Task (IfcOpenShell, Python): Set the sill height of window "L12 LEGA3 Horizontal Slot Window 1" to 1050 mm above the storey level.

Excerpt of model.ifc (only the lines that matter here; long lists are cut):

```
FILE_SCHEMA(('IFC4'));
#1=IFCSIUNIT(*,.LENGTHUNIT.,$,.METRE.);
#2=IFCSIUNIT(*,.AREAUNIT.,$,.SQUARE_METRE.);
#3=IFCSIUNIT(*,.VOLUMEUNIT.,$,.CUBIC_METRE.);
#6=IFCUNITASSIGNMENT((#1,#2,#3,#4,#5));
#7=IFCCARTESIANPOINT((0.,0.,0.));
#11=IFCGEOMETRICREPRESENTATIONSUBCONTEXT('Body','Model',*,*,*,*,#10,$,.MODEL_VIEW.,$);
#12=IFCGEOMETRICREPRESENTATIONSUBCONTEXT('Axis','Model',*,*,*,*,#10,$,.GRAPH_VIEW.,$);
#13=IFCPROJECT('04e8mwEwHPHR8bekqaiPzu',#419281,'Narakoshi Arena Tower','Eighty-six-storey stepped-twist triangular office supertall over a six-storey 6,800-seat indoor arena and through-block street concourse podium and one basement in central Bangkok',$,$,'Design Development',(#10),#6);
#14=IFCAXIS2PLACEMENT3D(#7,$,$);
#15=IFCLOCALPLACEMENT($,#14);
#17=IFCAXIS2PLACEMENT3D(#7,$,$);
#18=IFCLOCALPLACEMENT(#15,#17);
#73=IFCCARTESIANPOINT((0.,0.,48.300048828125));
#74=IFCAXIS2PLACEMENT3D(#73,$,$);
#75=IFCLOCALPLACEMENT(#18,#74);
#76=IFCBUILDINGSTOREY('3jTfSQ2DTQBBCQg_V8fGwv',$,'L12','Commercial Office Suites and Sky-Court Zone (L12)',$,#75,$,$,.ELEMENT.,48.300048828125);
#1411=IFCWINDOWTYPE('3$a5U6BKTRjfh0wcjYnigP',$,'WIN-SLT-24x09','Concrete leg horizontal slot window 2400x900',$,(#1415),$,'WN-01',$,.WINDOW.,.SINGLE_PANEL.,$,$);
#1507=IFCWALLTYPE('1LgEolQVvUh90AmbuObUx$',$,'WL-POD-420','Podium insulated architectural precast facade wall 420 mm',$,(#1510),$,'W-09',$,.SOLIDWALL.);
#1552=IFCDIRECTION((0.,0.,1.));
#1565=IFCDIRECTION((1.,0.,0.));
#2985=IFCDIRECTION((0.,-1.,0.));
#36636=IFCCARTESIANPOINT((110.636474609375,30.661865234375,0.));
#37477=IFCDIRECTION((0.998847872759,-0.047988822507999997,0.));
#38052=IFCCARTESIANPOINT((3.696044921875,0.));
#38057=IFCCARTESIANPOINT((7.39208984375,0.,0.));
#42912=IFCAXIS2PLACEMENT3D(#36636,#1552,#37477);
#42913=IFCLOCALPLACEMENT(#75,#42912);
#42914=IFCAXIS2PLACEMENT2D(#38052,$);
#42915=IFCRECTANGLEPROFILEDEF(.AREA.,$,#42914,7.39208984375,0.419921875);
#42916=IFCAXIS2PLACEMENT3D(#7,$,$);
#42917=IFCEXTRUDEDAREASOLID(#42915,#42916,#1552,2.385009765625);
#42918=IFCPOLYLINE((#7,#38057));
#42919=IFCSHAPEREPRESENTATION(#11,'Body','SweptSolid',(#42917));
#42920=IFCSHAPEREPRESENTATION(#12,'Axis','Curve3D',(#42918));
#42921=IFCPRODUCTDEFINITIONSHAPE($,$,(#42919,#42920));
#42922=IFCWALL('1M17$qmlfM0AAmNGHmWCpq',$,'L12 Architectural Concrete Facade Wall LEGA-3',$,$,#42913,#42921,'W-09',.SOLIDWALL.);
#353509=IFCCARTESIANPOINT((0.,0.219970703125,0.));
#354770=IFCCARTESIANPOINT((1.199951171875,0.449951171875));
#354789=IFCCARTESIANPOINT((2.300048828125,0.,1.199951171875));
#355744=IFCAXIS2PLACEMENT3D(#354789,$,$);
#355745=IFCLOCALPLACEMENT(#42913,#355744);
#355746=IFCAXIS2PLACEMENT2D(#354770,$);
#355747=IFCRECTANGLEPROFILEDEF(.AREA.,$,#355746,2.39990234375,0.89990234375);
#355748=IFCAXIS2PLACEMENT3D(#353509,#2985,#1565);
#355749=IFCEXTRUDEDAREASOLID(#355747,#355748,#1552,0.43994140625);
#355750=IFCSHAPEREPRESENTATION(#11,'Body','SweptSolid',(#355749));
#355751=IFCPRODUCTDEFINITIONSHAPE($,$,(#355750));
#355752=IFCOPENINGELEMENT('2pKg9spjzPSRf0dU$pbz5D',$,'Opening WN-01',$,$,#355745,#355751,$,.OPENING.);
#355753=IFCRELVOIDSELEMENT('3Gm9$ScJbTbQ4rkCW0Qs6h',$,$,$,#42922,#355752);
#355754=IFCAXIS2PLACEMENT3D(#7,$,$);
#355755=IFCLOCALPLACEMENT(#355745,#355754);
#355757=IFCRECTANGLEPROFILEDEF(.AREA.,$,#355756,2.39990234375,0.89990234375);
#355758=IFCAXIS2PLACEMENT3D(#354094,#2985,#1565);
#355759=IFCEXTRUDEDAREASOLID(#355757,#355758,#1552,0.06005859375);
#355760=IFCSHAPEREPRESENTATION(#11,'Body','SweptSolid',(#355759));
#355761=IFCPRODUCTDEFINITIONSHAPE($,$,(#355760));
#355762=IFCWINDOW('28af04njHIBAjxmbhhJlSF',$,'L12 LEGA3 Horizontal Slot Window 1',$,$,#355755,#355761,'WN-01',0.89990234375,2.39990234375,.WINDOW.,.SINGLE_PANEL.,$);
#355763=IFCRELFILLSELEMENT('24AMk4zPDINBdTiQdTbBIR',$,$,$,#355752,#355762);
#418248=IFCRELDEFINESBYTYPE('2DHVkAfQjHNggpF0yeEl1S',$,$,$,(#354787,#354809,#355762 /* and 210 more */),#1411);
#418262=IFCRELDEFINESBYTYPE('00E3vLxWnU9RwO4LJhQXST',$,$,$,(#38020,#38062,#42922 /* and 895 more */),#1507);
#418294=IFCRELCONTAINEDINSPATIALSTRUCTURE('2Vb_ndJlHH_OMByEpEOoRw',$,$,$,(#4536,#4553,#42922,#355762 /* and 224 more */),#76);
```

```python
import numpy as np
import ifcopenshell
import ifcopenshell.api.geometry
import ifcopenshell.geom
import ifcopenshell.util.element
import ifcopenshell.util.placement
import ifcopenshell.util.shape
import ifcopenshell.util.unit

model = ifcopenshell.open("model.ifc")
unit_scale = ifcopenshell.util.unit.calculate_unit_scale(model)

window = model.by_guid("28af04njHIBAjxmbhhJlSF")
opening = window.FillsVoids[0].RelatingOpeningElement
storey = ifcopenshell.util.element.get_container(window, ifc_class="IfcBuildingStorey")
level = ifcopenshell.util.placement.get_local_placement(storey.ObjectPlacement)[2, 3]

# The opening's origin need not be at the sill, so measure its lowest point.
shape = ifcopenshell.geom.create_shape(ifcopenshell.geom.settings(), opening)
bottom = ifcopenshell.util.shape.get_shape_bottom_elevation(shape, shape.geometry) / unit_scale
dz = level + 1.05 / unit_scale - bottom

shift = np.array([0.0, 0.0, dz])
# The window is placed relative to its opening, so it follows when the opening moves.
matrix = ifcopenshell.util.placement.get_local_placement(opening.ObjectPlacement)
matrix[:3, 3] += shift
ifcopenshell.api.geometry.edit_object_placement(
    model, product=opening, matrix=matrix, is_si=False, should_transform_children=True
)

print(f"moved by {dz * unit_scale:+.3f} m")

model.write("model_rev.ifc")
```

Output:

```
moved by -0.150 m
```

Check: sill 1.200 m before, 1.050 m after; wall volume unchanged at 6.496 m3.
